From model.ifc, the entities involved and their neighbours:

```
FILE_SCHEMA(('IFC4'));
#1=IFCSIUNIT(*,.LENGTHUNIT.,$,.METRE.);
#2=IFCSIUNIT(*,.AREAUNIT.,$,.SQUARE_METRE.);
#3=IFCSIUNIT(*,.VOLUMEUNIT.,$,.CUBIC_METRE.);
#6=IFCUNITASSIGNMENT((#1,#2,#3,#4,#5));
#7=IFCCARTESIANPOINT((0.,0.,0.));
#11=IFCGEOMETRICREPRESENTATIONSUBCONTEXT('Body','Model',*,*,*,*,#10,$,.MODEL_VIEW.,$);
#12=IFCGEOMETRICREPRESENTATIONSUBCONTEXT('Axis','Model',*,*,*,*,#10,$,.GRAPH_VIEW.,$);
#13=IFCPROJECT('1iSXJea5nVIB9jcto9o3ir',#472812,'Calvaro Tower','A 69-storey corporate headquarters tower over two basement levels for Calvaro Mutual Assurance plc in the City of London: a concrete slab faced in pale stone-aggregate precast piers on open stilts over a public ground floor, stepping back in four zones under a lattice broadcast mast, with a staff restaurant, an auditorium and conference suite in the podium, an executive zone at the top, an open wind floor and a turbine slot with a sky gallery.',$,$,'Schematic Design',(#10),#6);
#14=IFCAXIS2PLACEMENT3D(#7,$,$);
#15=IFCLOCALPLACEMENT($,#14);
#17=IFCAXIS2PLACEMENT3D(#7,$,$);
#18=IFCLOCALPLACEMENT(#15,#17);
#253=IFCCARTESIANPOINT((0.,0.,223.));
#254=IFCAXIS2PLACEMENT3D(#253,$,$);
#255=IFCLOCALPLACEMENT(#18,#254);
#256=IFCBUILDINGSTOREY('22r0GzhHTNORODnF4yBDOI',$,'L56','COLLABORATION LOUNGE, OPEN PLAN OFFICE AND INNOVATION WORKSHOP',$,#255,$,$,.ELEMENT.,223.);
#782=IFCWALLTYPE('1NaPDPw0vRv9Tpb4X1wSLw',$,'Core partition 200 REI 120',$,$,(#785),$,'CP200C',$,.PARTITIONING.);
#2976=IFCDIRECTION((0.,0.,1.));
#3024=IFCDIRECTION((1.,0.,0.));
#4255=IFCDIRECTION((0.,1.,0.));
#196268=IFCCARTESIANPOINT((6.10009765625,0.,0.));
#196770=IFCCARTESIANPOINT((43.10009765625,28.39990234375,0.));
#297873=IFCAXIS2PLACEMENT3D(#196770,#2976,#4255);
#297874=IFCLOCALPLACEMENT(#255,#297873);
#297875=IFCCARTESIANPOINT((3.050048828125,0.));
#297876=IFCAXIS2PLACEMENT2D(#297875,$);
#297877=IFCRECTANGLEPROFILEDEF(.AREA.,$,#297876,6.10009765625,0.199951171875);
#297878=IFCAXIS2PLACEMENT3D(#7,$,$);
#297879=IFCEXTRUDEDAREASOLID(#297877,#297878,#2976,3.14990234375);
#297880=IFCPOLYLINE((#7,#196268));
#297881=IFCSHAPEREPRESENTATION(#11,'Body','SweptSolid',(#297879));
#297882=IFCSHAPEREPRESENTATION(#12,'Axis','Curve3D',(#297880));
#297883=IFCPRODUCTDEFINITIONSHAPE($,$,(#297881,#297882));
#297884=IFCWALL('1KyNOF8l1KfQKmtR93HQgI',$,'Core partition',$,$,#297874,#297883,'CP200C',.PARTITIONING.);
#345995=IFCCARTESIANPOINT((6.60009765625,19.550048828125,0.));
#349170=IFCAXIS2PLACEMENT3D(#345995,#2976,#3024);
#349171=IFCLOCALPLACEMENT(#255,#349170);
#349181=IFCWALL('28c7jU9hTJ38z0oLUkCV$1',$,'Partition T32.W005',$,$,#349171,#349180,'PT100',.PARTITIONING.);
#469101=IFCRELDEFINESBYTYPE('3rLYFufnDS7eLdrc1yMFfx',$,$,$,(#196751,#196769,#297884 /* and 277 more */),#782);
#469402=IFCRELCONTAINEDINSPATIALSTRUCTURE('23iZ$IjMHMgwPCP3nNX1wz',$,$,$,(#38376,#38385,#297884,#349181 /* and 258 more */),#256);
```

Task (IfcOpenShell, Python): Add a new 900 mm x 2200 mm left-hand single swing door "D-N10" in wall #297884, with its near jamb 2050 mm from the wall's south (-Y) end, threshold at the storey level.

```python
import numpy as np
import ifcopenshell
import ifcopenshell.api.feature
import ifcopenshell.api.geometry
import ifcopenshell.api.root
import ifcopenshell.api.spatial
import ifcopenshell.geom
import ifcopenshell.util.element
import ifcopenshell.util.placement
import ifcopenshell.util.representation
import ifcopenshell.util.shape
import ifcopenshell.util.unit

model = ifcopenshell.open("model.ifc")
unit_scale = ifcopenshell.util.unit.calculate_unit_scale(model)
settings = ifcopenshell.geom.settings()


def volume(element):
    """Net volume in cubic metres, openings subtracted."""
    shape = ifcopenshell.geom.create_shape(settings, element)
    return ifcopenshell.util.shape.get_volume(shape.geometry)


wall = model.by_guid("1KyNOF8l1KfQKmtR93HQgI")
storey = ifcopenshell.util.element.get_container(wall, ifc_class="IfcBuildingStorey")
context = ifcopenshell.util.representation.get_context(model, "Model", "Body", "MODEL_VIEW")
before = volume(wall)

width, height, from_end, sill = 0.9, 2.2, 2.05, 0.0  # metres

# The wall runs along its own X axis, and the end named is its -X end.
wall_shape = ifcopenshell.geom.create_shape(settings, wall)
x, y, z = ifcopenshell.util.shape.get_vertices(wall_shape.geometry).T
start = x.min() + from_end
face, thickness = float(y.min()), float(y.max() - y.min())
wall_matrix = ifcopenshell.util.placement.get_local_placement(wall.ObjectPlacement)
level = ifcopenshell.util.placement.get_local_placement(storey.ObjectPlacement)[2, 3]


def in_wall(x, y):
    """Placement at x, y metres in the wall's axes, at sill height."""
    matrix = wall_matrix.copy()
    matrix[:, 3] = wall_matrix @ np.array([x / unit_scale, y / unit_scale, 0.0, 1.0])
    matrix[2, 3] = level + sill / unit_scale
    return matrix


# Opening: a box that overshoots both wall faces by 50 mm.
opening = ifcopenshell.api.root.create_entity(model, ifc_class="IfcOpeningElement", predefined_type="OPENING")
box = ifcopenshell.api.geometry.add_wall_representation(
    model, context=context, length=width, height=height, thickness=thickness + 0.1
)
ifcopenshell.api.geometry.assign_representation(model, product=opening, representation=box)
ifcopenshell.api.geometry.edit_object_placement(model, product=opening, matrix=in_wall(start, face - 0.05), is_si=False)
ifcopenshell.api.feature.add_feature(model, feature=opening, element=wall)

door = ifcopenshell.api.root.create_entity(model, ifc_class="IfcDoor", name="D-N10", predefined_type="DOOR")
door.OverallWidth, door.OverallHeight = width / unit_scale, height / unit_scale
door.OperationType = "SINGLE_SWING_LEFT"
body = ifcopenshell.api.geometry.add_door_representation(
    model,
    context=context,
    overall_width=door.OverallWidth,
    overall_height=door.OverallHeight,
    operation_type="SINGLE_SWING_LEFT",
    lining_properties={"LiningDepth": thickness / unit_scale, "ThresholdDepth": thickness / unit_scale},
)
ifcopenshell.api.geometry.assign_representation(model, product=door, representation=body)
ifcopenshell.api.spatial.assign_container(model, products=[door], relating_structure=storey)
ifcopenshell.api.feature.add_filling(model, opening=opening, element=door)

# The lining spans the wall, so the door starts at the wall face.
ifcopenshell.api.geometry.edit_object_placement(model, product=door, matrix=in_wall(start, face), is_si=False)

after = volume(wall)

print(f"wall volume {before:.3f} -> {after:.3f} m3")

model.write("model-out.ifc")
```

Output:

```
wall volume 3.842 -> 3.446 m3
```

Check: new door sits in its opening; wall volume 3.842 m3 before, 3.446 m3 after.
